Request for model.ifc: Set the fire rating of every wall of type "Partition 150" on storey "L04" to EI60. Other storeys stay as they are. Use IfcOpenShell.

First a look at what the model holds.

```python
import ifcopenshell
import ifcopenshell.util.element

model = ifcopenshell.open("model.ifc")
print(model.schema)
storey = next(s for s in model.by_type("IfcBuildingStorey") if s.Name == "L04")
walls = [e for e in ifcopenshell.util.element.get_decomposition(storey) if e.is_a("IfcWall")]
seen = {}
for e in walls:
    element_type = ifcopenshell.util.element.get_type(e)
    key = (element_type.Name if element_type != e and element_type else None, ifcopenshell.util.element.get_pset(e, "Pset_WallCommon", "FireRating"))
    seen[key] = seen.get(key, 0) + 1
for (name, value), count in sorted(seen.items(), key=str):
    print(count, "x", name, "|", value)
```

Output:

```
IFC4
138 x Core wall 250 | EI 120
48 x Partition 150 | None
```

```python
import ifcopenshell
import ifcopenshell.api.pset
import ifcopenshell.util.element

model = ifcopenshell.open("model.ifc")

storey = next(s for s in model.by_type("IfcBuildingStorey") if s.Name == "L04")
walls = [e for e in ifcopenshell.util.element.get_decomposition(storey) if e.is_a("IfcWall")]

count = 0
for e in walls:
    element_type = ifcopenshell.util.element.get_type(e)
    if element_type in (None, e) or element_type.Name != "Partition 150":
        continue
    # add_pset returns the element's existing set when there is one.
    pset = ifcopenshell.api.pset.add_pset(model, product=e, name="Pset_WallCommon")
    ifcopenshell.api.pset.edit_pset(model, pset=pset, properties={"FireRating": "EI60"})
    count += 1

print(count, "walls updated")

model.write("model_updated.ifc")
```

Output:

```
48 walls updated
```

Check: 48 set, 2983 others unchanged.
